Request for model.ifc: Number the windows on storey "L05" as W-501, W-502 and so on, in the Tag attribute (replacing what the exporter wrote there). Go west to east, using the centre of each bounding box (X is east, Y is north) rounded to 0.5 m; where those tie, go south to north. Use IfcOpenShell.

First a look at what the model holds.

```python
import ifcopenshell
import ifcopenshell.util.element
import ifcopenshell.util.placement

model = ifcopenshell.open("model.ifc")
print(model.schema)
storey = next(s for s in model.by_type("IfcBuildingStorey") if s.Name == "L05")
windows = [e for e in ifcopenshell.util.element.get_decomposition(storey) if e.is_a("IfcWindow")]
for e in sorted(windows, key=lambda e: e.id()):
    origin = ifcopenshell.util.placement.get_local_placement(e.ObjectPlacement)[:3, 3]
    print(e.id(), e.Tag, e.Name, origin.round(2) + 0.0, sep=" | ")
```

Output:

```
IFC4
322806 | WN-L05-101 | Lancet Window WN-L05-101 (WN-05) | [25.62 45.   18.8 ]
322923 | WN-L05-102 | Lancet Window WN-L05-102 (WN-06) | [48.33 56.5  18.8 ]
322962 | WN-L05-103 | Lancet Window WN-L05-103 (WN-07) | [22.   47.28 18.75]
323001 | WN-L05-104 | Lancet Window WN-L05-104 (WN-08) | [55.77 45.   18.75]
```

```python
import ifcopenshell
import ifcopenshell.geom
import ifcopenshell.util.element
import ifcopenshell.util.shape

model = ifcopenshell.open("model.ifc")
settings = ifcopenshell.geom.settings()
settings.set("use-world-coords", True)


def centre(element):
    shape = ifcopenshell.geom.create_shape(settings, element)
    return ifcopenshell.util.shape.get_bbox_centroid(shape.geometry)


storey = next(s for s in model.by_type("IfcBuildingStorey") if s.Name == "L05")
windows = [e for e in ifcopenshell.util.element.get_decomposition(storey) if e.is_a("IfcWindow")]

# Insertion points can sit at a corner or the storey origin, so sort by the geometry (in metres).
centres = {e: centre(e) for e in windows}
windows.sort(key=lambda e: (round(centres[e][0] / 0.5), centres[e][1]))

for i, e in enumerate(windows, start=1):
    number = f"W-5{i:02d}"
    e.Tag = number
    print(e.id(), number)

model.write("model_edited.ifc")
```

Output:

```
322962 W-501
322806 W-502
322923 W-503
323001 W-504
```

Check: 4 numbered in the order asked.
